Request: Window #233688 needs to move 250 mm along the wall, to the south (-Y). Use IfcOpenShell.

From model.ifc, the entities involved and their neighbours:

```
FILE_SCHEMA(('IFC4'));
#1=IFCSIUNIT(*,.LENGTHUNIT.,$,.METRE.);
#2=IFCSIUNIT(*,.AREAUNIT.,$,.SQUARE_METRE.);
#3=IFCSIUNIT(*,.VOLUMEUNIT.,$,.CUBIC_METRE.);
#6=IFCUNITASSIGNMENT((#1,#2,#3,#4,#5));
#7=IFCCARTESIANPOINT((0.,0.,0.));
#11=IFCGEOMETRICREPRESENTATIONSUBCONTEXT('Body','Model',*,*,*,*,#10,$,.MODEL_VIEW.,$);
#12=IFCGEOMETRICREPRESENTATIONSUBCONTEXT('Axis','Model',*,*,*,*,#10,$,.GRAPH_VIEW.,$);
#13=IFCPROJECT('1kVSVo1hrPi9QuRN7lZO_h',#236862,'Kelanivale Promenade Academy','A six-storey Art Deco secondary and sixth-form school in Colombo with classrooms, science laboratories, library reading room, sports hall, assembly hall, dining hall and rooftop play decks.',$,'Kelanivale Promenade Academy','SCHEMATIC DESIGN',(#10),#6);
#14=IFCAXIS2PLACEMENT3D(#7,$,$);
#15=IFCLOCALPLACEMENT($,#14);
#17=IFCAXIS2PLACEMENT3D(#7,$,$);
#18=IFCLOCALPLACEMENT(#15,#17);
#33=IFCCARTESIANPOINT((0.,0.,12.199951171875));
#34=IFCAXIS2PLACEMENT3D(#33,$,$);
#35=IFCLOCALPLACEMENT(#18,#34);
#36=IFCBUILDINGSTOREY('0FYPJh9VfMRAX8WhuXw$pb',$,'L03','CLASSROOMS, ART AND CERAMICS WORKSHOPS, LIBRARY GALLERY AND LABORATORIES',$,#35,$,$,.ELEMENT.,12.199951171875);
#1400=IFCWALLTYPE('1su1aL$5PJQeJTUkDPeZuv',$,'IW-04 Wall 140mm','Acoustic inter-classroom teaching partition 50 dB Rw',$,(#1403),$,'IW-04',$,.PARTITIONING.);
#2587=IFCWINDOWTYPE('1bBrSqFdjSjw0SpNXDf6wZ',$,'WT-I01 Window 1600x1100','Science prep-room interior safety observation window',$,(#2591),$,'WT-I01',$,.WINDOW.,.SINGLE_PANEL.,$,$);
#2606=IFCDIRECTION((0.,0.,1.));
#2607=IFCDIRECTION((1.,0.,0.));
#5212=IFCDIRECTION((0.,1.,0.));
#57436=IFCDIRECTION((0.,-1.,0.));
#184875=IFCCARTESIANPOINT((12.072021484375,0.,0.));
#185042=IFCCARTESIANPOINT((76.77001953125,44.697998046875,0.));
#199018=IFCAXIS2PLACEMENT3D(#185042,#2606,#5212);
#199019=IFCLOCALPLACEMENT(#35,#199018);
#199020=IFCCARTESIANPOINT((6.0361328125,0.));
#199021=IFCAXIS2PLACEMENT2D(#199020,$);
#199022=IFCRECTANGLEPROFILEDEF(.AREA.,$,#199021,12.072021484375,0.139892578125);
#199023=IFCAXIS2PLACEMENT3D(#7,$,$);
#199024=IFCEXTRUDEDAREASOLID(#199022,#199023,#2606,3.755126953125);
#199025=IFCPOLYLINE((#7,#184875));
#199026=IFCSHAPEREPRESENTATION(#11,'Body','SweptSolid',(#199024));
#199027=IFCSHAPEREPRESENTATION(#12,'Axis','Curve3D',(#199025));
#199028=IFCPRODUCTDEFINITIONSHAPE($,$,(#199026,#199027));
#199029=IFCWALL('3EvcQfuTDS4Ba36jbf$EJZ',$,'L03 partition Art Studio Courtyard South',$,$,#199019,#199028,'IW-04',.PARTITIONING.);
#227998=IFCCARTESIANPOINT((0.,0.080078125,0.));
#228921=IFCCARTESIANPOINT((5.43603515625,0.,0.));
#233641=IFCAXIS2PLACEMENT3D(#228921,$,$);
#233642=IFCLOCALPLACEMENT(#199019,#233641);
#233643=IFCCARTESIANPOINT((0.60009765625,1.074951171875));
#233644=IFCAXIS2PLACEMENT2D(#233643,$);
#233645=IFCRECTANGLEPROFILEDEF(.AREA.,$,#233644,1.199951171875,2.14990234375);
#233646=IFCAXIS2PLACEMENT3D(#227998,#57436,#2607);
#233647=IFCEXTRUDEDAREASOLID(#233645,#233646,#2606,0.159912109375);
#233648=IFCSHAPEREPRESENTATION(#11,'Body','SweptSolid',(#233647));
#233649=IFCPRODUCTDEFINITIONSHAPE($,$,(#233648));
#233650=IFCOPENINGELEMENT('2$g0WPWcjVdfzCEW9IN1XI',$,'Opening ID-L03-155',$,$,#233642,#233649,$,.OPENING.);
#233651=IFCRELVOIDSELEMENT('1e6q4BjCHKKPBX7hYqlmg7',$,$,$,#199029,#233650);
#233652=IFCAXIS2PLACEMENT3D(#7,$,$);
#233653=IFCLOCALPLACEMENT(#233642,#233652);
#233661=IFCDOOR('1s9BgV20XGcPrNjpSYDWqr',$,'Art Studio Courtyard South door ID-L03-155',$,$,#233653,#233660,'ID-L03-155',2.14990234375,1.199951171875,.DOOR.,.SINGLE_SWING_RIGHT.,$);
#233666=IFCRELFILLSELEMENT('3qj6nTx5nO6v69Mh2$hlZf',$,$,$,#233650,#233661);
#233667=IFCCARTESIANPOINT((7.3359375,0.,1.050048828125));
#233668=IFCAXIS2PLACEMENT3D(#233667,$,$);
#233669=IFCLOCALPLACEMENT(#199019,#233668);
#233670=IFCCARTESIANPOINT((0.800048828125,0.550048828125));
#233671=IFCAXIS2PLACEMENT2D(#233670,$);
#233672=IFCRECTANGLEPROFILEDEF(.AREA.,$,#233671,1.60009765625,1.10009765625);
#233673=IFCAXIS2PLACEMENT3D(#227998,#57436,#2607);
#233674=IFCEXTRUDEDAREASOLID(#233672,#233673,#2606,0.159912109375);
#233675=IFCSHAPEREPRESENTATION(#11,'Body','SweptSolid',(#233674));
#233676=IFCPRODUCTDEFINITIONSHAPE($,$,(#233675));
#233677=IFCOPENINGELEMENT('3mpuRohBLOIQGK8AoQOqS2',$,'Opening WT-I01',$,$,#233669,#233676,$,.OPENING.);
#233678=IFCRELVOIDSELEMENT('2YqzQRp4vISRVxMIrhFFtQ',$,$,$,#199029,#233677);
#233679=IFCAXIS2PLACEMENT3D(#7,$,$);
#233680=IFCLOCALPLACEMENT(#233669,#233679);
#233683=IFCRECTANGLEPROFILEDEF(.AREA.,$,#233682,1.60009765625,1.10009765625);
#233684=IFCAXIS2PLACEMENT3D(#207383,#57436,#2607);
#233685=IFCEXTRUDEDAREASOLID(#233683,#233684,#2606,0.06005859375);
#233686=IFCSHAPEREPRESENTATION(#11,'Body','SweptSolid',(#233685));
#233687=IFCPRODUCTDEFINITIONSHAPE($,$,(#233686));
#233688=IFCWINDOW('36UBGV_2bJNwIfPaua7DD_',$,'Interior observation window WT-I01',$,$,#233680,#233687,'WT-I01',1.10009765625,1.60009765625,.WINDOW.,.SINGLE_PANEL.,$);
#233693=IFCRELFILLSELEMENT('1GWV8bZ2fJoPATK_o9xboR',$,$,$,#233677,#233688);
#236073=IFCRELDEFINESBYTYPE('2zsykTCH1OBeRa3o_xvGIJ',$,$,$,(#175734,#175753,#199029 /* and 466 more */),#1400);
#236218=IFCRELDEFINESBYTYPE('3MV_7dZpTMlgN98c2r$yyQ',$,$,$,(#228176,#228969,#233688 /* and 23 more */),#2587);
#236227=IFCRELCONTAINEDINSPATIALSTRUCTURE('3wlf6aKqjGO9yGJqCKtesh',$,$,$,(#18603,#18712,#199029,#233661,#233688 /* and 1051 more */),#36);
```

```python
import ifcopenshell
import ifcopenshell.api.geometry
import ifcopenshell.util.placement
import ifcopenshell.util.unit

model = ifcopenshell.open("model.ifc")
unit_scale = ifcopenshell.util.unit.calculate_unit_scale(model)

window = model.by_guid("36UBGV_2bJNwIfPaua7DD_")
opening = window.FillsVoids[0].RelatingOpeningElement
wall = opening.VoidsElements[0].RelatingBuildingElement

wall_matrix = ifcopenshell.util.placement.get_local_placement(wall.ObjectPlacement)
shift = wall_matrix[:3, 0] * -0.25 / unit_scale
before = ifcopenshell.util.placement.get_local_placement(window.ObjectPlacement)[:3, 3].copy()

# The window is placed relative to its opening, so it follows when the opening moves.
matrix = ifcopenshell.util.placement.get_local_placement(opening.ObjectPlacement)
matrix[:3, 3] += shift
ifcopenshell.api.geometry.edit_object_placement(
    model, product=opening, matrix=matrix, is_si=False, should_transform_children=True
)

after = ifcopenshell.util.placement.get_local_placement(window.ObjectPlacement)[:3, 3]
print("window moved by", (after - before).round(3) + 0.0)

model.write("model_rev.ifc")
```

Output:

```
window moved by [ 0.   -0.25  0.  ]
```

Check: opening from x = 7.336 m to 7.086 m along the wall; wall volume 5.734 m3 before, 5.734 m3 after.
